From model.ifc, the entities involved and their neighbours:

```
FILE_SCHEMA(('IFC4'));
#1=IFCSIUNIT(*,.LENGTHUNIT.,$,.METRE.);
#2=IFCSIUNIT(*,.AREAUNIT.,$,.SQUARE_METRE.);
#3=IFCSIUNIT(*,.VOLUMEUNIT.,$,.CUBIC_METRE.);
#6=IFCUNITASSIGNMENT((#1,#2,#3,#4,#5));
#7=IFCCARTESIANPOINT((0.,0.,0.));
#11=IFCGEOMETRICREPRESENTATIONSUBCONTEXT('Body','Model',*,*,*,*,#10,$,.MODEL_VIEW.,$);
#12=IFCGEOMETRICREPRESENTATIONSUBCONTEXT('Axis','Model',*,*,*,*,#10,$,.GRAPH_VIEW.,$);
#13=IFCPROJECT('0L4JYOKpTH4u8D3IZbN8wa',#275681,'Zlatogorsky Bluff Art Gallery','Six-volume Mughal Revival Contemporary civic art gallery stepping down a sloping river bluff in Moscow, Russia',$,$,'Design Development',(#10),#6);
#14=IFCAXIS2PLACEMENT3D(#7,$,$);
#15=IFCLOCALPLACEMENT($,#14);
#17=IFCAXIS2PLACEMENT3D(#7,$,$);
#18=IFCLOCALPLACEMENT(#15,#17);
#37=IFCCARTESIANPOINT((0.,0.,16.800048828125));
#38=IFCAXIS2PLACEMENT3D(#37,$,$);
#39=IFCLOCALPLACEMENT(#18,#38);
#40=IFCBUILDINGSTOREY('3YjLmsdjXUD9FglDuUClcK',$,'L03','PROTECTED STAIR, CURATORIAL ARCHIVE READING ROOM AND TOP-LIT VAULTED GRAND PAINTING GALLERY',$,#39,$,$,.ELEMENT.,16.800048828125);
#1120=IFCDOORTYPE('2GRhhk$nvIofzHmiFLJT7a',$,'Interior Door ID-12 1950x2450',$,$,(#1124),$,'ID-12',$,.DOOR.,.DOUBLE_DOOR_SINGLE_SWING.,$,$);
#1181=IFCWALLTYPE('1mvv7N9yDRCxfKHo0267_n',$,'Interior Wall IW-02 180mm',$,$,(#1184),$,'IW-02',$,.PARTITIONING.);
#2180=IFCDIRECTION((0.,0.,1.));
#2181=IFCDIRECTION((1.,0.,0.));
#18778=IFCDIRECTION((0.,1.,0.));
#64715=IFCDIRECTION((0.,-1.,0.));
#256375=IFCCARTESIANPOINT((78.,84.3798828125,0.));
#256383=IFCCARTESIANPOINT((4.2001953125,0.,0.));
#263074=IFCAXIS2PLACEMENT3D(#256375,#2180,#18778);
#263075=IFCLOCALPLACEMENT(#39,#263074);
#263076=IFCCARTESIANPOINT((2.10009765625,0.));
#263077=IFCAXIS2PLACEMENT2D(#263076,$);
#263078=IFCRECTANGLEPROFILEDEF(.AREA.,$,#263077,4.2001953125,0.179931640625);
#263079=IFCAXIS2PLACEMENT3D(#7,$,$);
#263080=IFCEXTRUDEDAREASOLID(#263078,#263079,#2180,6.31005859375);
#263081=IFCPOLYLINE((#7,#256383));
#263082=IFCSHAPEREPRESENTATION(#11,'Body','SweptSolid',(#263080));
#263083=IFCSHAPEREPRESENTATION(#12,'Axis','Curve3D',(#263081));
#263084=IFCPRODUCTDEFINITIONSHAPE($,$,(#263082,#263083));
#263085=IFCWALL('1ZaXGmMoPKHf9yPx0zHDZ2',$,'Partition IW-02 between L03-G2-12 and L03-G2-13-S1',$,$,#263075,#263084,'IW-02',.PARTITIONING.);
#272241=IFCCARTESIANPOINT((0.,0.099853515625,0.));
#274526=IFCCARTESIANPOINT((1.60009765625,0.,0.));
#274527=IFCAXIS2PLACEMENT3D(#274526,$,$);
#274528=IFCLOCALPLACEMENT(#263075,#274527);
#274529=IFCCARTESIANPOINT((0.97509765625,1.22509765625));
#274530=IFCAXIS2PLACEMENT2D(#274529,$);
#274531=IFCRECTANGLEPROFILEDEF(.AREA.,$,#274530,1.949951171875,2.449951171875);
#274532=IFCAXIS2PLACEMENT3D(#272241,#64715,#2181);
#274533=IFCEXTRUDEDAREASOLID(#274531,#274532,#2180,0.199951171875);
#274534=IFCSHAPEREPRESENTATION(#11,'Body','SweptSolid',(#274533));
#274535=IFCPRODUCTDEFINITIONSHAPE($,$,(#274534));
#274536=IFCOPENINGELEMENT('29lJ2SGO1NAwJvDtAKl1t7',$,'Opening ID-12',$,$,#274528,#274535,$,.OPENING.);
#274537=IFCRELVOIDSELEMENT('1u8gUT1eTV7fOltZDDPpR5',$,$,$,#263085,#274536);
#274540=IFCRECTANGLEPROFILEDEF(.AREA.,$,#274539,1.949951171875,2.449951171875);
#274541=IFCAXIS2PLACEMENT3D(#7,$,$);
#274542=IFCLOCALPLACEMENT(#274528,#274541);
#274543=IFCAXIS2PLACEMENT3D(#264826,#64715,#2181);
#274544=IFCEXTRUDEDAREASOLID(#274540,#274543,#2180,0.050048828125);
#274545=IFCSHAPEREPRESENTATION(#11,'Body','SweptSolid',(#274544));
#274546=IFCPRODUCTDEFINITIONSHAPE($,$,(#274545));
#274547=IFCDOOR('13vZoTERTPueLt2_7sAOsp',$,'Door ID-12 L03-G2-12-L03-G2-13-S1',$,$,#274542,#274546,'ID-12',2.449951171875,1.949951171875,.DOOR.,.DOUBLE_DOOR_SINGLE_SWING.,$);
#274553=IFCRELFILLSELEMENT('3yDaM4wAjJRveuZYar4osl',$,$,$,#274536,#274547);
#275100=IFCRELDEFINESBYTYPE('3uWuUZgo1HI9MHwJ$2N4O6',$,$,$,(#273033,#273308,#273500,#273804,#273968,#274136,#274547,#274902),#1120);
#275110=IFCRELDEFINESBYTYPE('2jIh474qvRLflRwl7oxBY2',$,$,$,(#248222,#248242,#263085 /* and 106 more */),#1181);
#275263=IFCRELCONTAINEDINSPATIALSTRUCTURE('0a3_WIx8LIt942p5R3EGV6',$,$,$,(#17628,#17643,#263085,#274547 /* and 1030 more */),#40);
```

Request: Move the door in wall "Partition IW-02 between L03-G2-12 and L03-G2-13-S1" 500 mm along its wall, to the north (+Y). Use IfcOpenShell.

```python
import ifcopenshell
import ifcopenshell.api.geometry
import ifcopenshell.util.placement
import ifcopenshell.util.unit

model = ifcopenshell.open("model.ifc")
unit_scale = ifcopenshell.util.unit.calculate_unit_scale(model)

door = model.by_id(274547)
opening = door.FillsVoids[0].RelatingOpeningElement
wall = opening.VoidsElements[0].RelatingBuildingElement

wall_matrix = ifcopenshell.util.placement.get_local_placement(wall.ObjectPlacement)
shift = wall_matrix[:3, 0] * 0.5 / unit_scale
before = ifcopenshell.util.placement.get_local_placement(door.ObjectPlacement)[:3, 3].copy()

# The door is placed relative to its opening, so it follows when the opening moves.
matrix = ifcopenshell.util.placement.get_local_placement(opening.ObjectPlacement)
matrix[:3, 3] += shift
ifcopenshell.api.geometry.edit_object_placement(
    model, product=opening, matrix=matrix, is_si=False, should_transform_children=True
)

after = ifcopenshell.util.placement.get_local_placement(door.ObjectPlacement)[:3, 3]
print("door moved by", (after - before).round(3) + 0.0)

model.write("model_rev.ifc")
```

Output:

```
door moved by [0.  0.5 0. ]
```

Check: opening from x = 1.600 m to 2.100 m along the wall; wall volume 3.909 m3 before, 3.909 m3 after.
